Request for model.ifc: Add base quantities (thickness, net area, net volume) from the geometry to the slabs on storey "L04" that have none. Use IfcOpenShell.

First a look at what the model holds.

```python
import ifcopenshell
import ifcopenshell.util.element
import ifcopenshell.util.unit

model = ifcopenshell.open("model.ifc")
print(model.schema)
for unit_type in ("LENGTHUNIT", "AREAUNIT", "VOLUMEUNIT"):
    print(unit_type, ifcopenshell.util.unit.calculate_unit_scale(model, unit_type))
storey = next(s for s in model.by_type("IfcBuildingStorey") if s.Name == "L04")
slabs = [e for e in ifcopenshell.util.element.get_decomposition(storey) if e.is_a("IfcSlab")]
for e in sorted(slabs, key=lambda e: e.id()):
    print(e.id(), e.is_a(), e.Name, list(ifcopenshell.util.element.get_psets(e, qtos_only=True)), sep=" | ")
```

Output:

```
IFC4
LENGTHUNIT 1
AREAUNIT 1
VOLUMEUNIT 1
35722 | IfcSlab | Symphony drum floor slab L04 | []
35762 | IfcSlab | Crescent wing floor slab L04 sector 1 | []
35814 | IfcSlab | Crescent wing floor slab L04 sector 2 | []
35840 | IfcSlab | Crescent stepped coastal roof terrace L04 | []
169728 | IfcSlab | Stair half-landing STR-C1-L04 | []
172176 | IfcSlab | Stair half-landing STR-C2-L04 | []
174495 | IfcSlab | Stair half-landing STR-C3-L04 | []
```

```python
import ifcopenshell
import ifcopenshell.api.pset
import ifcopenshell.geom
import ifcopenshell.util.element
import ifcopenshell.util.shape
import ifcopenshell.util.unit

model = ifcopenshell.open("model.ifc")
unit_scale = ifcopenshell.util.unit.calculate_unit_scale(model)
area_scale = ifcopenshell.util.unit.calculate_unit_scale(model, "AREAUNIT")
volume_scale = ifcopenshell.util.unit.calculate_unit_scale(model, "VOLUMEUNIT")
settings = ifcopenshell.geom.settings()

storey = next(s for s in model.by_type("IfcBuildingStorey") if s.Name == "L04")
slabs = [e for e in ifcopenshell.util.element.get_decomposition(storey) if e.is_a("IfcSlab")]

for e in sorted(slabs, key=lambda e: e.id()):
    if ifcopenshell.util.element.get_psets(e, qtos_only=True, should_inherit=False):
        continue
    # Geometry comes back in metres, in the element's own axes.
    shape = ifcopenshell.geom.create_shape(settings, e)
    values = {
        "Width": ifcopenshell.util.shape.get_z(shape.geometry) / unit_scale,
        "NetArea": ifcopenshell.util.shape.get_footprint_area(shape.geometry) / area_scale,
        "NetVolume": ifcopenshell.util.shape.get_volume(shape.geometry) / volume_scale,
    }
    qto = ifcopenshell.api.pset.add_qto(model, product=e, name="Qto_SlabBaseQuantities")
    ifcopenshell.api.pset.edit_qto(model, qto=qto, properties=values)
    print(e.id(), {k: round(v, 3) for k, v in values.items()})

model.write("model_edited.ifc")
```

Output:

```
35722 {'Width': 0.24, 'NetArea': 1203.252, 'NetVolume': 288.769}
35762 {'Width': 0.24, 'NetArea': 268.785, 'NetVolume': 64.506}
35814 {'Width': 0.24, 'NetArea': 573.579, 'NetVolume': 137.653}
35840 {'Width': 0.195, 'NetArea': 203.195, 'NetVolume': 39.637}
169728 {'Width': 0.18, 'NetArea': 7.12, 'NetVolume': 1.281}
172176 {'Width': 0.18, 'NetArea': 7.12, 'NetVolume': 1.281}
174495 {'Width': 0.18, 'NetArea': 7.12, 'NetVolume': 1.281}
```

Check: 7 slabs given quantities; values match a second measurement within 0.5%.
